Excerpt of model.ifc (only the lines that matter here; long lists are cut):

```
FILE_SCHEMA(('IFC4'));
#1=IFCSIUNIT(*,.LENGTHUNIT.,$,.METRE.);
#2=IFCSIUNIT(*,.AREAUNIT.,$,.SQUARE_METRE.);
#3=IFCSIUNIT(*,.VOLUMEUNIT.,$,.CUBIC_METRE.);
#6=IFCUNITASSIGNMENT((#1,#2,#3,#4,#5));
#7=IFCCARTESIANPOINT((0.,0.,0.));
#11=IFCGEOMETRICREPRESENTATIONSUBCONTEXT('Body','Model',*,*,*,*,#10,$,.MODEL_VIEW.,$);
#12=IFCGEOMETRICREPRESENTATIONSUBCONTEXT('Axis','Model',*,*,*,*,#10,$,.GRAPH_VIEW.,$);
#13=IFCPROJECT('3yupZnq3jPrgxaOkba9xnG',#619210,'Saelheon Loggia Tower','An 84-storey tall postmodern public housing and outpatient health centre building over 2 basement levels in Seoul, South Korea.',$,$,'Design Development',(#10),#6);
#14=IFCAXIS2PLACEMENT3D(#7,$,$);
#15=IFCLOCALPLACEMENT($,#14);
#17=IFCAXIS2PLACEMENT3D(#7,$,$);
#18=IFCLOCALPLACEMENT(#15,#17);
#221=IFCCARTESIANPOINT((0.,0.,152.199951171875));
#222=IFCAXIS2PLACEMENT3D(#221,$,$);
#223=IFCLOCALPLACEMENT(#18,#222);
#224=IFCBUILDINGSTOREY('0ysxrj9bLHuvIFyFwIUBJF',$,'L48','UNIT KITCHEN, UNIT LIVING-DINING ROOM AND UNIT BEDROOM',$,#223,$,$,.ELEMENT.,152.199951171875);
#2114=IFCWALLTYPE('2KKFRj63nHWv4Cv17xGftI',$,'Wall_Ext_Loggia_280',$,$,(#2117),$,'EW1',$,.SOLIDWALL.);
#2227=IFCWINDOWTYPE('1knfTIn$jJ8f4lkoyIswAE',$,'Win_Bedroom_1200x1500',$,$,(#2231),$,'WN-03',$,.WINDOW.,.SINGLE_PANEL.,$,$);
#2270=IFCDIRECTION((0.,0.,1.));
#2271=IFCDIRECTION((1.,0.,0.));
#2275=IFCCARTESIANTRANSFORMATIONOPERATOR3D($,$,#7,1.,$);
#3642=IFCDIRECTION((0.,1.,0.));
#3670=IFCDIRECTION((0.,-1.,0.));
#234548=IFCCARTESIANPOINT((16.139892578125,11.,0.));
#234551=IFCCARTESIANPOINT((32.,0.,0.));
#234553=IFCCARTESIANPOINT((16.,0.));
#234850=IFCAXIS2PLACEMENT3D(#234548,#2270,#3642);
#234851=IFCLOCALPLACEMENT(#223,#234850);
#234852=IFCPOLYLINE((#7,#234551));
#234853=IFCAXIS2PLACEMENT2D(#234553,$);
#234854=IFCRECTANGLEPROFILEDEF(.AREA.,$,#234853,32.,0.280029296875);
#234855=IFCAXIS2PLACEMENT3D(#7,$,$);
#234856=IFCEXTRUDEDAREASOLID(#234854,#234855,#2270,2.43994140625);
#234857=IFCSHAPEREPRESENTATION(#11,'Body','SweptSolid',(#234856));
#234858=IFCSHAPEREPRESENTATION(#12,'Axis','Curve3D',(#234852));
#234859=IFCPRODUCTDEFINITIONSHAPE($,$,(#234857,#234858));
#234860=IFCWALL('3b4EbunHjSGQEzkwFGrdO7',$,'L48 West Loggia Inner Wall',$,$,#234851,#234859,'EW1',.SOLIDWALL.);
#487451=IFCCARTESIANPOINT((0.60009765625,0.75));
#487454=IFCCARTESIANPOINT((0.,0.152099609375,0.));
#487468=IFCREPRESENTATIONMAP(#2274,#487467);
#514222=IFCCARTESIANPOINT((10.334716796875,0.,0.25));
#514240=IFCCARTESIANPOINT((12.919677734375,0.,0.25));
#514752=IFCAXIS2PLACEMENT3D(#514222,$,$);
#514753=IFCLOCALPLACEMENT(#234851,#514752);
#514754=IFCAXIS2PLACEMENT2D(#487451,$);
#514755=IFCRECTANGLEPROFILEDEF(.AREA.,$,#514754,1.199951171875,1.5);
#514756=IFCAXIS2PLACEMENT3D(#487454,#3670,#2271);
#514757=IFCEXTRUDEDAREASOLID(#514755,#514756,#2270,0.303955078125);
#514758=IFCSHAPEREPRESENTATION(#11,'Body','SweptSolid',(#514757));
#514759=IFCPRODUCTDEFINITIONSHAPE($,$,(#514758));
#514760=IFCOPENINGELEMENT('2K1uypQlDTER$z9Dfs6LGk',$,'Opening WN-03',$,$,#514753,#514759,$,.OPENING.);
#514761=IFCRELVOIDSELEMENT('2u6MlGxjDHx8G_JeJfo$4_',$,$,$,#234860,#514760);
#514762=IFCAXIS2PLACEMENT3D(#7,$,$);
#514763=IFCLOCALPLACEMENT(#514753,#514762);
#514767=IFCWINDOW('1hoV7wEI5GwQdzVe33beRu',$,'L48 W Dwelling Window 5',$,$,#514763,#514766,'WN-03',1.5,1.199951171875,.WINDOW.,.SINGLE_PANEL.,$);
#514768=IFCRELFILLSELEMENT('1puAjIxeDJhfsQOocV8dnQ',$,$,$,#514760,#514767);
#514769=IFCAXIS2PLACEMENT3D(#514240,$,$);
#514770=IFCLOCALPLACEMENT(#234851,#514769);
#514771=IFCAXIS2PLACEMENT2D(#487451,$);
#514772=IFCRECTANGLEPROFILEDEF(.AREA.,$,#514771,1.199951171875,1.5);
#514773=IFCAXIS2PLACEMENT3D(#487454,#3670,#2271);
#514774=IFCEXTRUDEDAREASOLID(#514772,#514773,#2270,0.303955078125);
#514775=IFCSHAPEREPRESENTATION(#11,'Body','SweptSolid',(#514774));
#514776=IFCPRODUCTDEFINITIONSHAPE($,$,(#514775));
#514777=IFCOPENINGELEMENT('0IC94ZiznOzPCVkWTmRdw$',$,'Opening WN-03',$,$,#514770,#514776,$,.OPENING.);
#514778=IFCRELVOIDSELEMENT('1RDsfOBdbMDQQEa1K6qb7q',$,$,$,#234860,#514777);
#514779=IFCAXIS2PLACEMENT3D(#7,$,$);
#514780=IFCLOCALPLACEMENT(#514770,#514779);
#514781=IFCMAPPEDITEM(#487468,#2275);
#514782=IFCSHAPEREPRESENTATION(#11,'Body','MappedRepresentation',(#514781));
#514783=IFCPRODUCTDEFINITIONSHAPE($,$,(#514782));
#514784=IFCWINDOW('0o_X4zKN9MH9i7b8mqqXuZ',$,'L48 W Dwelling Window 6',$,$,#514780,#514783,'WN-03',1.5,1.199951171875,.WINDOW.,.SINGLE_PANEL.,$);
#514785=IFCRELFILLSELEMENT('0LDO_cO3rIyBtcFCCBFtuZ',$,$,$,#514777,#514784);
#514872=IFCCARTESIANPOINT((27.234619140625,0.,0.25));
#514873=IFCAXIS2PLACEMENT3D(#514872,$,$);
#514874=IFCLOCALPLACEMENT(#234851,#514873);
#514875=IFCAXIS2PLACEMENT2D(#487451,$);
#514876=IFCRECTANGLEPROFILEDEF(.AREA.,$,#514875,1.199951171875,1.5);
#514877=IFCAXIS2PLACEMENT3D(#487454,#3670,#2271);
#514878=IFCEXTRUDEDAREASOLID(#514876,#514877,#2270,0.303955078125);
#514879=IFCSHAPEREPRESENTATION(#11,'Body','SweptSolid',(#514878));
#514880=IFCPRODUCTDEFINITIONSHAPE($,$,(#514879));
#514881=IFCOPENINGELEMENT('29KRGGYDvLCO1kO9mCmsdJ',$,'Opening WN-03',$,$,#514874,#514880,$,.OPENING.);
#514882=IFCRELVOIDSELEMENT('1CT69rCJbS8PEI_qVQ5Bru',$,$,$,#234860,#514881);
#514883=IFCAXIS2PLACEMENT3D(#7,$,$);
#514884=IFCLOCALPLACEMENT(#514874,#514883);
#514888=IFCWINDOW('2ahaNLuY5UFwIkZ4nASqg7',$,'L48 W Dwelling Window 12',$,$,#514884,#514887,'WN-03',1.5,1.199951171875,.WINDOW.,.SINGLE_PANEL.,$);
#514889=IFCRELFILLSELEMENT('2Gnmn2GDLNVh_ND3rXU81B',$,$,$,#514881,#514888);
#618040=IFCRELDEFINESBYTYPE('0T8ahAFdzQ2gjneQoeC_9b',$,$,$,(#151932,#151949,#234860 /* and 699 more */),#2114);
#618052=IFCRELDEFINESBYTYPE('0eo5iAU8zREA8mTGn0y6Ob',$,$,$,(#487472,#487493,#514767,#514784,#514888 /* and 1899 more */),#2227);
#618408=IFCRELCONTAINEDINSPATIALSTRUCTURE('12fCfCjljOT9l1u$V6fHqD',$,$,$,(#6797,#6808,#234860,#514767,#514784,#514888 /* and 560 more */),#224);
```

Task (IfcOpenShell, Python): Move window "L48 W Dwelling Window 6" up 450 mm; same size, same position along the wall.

```python
import numpy as np
import ifcopenshell
import ifcopenshell.api.geometry
import ifcopenshell.util.placement
import ifcopenshell.util.unit

model = ifcopenshell.open("model.ifc")
unit_scale = ifcopenshell.util.unit.calculate_unit_scale(model)

window = model.by_guid("0o_X4zKN9MH9i7b8mqqXuZ")
opening = window.FillsVoids[0].RelatingOpeningElement
dz = 0.45

shift = np.array([0.0, 0.0, dz])
# The window is placed relative to its opening, so it follows when the opening moves.
matrix = ifcopenshell.util.placement.get_local_placement(opening.ObjectPlacement)
matrix[:3, 3] += shift
ifcopenshell.api.geometry.edit_object_placement(
    model, product=opening, matrix=matrix, is_si=False, should_transform_children=True
)

print(f"moved by {dz * unit_scale:+.3f} m")

model.write("model_v2.ifc")
```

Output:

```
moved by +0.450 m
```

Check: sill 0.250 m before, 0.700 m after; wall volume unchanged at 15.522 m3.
